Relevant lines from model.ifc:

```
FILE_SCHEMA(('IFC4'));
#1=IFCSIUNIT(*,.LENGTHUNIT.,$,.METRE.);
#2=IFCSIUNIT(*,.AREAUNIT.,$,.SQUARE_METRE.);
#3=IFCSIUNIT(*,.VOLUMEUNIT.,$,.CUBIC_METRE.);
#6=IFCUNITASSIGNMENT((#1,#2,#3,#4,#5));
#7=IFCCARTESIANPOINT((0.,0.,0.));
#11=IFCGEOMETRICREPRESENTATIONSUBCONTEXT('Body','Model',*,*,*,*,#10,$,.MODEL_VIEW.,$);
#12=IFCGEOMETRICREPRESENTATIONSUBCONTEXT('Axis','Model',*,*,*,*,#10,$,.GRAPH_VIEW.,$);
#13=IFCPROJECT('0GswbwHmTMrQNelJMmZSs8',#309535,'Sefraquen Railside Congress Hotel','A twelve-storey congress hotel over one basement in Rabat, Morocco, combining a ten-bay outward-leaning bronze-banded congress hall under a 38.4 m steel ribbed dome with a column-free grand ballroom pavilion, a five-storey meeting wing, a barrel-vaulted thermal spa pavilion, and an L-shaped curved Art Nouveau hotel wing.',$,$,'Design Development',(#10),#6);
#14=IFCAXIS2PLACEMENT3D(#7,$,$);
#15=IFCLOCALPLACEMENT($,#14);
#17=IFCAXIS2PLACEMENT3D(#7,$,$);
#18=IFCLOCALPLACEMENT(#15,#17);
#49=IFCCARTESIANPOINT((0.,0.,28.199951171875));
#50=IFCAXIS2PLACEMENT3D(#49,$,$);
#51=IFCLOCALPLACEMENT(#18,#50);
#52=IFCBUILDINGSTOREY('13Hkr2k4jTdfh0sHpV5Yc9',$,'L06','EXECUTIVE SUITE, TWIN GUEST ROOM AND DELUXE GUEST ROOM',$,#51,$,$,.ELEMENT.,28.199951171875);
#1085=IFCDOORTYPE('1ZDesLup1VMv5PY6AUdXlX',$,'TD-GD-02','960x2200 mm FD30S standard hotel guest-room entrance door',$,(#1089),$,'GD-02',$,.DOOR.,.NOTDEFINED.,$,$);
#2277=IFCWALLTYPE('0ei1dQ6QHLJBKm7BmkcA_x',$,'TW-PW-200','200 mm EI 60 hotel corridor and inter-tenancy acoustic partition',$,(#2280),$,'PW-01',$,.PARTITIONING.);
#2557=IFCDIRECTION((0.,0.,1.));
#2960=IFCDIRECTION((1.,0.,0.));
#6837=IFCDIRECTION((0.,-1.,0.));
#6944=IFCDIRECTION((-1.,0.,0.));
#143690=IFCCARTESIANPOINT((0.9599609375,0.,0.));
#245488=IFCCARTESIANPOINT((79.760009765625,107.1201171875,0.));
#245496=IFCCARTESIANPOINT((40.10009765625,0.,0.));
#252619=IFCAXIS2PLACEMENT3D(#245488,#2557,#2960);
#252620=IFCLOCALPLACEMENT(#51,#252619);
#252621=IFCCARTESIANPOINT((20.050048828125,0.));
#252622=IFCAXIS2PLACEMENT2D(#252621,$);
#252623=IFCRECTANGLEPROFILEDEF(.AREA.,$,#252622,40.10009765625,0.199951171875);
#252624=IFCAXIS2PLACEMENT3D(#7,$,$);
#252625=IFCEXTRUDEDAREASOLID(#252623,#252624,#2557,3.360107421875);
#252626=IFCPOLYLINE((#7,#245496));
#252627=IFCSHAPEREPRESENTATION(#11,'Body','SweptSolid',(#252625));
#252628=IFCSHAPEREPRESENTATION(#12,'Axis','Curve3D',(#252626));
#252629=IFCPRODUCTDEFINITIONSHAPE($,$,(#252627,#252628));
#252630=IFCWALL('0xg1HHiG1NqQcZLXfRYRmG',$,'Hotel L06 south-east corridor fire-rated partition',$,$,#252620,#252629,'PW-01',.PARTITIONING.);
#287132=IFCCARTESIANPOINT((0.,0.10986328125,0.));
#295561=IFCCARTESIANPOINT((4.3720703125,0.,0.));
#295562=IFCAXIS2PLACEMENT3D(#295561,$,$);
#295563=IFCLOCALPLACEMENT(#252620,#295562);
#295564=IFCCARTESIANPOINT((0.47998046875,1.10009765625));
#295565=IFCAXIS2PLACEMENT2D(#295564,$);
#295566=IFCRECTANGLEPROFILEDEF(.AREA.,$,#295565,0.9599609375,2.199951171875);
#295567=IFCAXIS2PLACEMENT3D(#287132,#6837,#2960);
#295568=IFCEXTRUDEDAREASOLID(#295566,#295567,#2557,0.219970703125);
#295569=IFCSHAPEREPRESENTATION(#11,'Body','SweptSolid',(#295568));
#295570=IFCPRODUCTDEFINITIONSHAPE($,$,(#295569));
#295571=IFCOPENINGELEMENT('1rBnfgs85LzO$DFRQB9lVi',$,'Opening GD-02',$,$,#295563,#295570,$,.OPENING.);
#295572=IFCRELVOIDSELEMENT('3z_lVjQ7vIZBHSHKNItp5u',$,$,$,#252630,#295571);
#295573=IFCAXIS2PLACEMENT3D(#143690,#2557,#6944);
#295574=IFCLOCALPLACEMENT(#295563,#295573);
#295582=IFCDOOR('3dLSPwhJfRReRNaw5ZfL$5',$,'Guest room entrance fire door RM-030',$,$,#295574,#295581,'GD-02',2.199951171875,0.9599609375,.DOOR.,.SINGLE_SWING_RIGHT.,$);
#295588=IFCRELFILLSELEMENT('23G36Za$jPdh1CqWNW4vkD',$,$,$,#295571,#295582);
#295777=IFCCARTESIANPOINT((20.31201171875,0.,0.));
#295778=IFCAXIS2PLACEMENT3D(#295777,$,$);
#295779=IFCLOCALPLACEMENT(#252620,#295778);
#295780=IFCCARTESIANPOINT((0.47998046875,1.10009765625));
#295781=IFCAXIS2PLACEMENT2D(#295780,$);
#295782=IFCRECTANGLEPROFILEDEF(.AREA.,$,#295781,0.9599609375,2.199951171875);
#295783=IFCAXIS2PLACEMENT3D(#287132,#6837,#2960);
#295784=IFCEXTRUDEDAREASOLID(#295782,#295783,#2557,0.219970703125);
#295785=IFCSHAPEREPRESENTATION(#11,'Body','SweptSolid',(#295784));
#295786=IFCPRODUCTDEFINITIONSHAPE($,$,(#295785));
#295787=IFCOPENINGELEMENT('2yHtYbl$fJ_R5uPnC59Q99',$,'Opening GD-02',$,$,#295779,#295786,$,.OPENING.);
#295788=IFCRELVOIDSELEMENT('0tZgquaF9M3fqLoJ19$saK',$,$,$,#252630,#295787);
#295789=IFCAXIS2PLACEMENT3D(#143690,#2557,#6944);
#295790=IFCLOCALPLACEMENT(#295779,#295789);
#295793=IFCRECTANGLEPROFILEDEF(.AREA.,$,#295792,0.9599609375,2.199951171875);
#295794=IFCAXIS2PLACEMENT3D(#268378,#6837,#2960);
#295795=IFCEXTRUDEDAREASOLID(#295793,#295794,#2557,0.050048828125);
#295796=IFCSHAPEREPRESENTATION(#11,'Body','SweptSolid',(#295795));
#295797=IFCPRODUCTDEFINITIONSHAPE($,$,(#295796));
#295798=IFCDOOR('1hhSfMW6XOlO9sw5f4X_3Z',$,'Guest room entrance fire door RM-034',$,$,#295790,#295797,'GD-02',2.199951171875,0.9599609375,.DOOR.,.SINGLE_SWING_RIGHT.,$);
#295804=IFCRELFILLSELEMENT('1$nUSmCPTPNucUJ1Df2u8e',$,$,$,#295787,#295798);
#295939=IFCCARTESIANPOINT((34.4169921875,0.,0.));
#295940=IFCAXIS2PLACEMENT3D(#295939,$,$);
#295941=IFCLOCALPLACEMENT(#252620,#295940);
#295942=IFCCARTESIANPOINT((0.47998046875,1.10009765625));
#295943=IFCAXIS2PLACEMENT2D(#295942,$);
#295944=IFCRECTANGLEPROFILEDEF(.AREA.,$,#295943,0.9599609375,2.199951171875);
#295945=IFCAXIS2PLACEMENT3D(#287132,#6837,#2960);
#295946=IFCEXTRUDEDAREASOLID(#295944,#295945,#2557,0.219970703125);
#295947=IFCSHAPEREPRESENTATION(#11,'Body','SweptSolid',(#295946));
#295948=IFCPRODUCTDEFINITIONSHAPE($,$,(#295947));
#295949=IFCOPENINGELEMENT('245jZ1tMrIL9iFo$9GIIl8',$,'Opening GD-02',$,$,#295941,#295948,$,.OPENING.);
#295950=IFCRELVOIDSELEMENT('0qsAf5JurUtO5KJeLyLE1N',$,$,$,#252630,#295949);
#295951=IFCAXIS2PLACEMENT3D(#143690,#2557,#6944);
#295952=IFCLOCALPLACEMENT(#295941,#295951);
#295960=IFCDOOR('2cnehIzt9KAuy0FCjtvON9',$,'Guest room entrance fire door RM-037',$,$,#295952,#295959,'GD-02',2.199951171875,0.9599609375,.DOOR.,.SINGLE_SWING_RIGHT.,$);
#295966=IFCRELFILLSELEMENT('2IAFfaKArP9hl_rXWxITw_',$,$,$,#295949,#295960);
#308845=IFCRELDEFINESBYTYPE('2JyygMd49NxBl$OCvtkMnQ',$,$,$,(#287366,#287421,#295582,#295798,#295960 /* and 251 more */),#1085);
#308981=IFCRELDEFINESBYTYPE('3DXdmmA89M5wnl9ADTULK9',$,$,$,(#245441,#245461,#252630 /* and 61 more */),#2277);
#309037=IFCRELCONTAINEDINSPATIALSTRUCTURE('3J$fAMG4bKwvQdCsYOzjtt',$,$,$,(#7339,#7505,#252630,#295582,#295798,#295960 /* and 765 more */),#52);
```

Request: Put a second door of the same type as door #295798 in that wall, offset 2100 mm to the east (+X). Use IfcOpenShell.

```python
import ifcopenshell
import ifcopenshell.api.feature
import ifcopenshell.api.geometry
import ifcopenshell.api.root
import ifcopenshell.geom
import ifcopenshell.util.element
import ifcopenshell.util.placement
import ifcopenshell.util.shape
import ifcopenshell.util.unit

model = ifcopenshell.open("model.ifc")
unit_scale = ifcopenshell.util.unit.calculate_unit_scale(model)
settings = ifcopenshell.geom.settings()


def volume(element):
    """Net volume in cubic metres, openings subtracted."""
    shape = ifcopenshell.geom.create_shape(settings, element)
    return ifcopenshell.util.shape.get_volume(shape.geometry)


door = model.by_guid("1hhSfMW6XOlO9sw5f4X_3Z")
opening = door.FillsVoids[0].RelatingOpeningElement
wall = opening.VoidsElements[0].RelatingBuildingElement
before = volume(wall)
shift = ifcopenshell.util.placement.get_local_placement(wall.ObjectPlacement)[:3, 0] * 2.1 / unit_scale

# copy_class copies the void relationship, type, container and properties, but no geometry.
new_opening = ifcopenshell.api.root.copy_class(model, product=opening)
new_opening.Representation = ifcopenshell.util.element.copy_deep(
    model, opening.Representation, exclude=["IfcGeometricRepresentationContext", "IfcRepresentationMap"]
)
new_door = ifcopenshell.api.root.copy_class(model, product=door)
new_door.Representation = ifcopenshell.util.element.copy_deep(
    model, door.Representation, exclude=["IfcGeometricRepresentationContext", "IfcRepresentationMap"]
)
new_door.Tag = None
ifcopenshell.api.feature.add_filling(model, opening=new_opening, element=new_door)

for old, new in ((opening, new_opening), (door, new_door)):
    matrix = ifcopenshell.util.placement.get_local_placement(old.ObjectPlacement)
    matrix[:3, 3] += shift
    ifcopenshell.api.geometry.edit_object_placement(model, product=new, matrix=matrix, is_si=False)

after = volume(wall)

print(f"wall volume {before:.3f} -> {after:.3f} m3")

model.write("model_v2.ifc")
```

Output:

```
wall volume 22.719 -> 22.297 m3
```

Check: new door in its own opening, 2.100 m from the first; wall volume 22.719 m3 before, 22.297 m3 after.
